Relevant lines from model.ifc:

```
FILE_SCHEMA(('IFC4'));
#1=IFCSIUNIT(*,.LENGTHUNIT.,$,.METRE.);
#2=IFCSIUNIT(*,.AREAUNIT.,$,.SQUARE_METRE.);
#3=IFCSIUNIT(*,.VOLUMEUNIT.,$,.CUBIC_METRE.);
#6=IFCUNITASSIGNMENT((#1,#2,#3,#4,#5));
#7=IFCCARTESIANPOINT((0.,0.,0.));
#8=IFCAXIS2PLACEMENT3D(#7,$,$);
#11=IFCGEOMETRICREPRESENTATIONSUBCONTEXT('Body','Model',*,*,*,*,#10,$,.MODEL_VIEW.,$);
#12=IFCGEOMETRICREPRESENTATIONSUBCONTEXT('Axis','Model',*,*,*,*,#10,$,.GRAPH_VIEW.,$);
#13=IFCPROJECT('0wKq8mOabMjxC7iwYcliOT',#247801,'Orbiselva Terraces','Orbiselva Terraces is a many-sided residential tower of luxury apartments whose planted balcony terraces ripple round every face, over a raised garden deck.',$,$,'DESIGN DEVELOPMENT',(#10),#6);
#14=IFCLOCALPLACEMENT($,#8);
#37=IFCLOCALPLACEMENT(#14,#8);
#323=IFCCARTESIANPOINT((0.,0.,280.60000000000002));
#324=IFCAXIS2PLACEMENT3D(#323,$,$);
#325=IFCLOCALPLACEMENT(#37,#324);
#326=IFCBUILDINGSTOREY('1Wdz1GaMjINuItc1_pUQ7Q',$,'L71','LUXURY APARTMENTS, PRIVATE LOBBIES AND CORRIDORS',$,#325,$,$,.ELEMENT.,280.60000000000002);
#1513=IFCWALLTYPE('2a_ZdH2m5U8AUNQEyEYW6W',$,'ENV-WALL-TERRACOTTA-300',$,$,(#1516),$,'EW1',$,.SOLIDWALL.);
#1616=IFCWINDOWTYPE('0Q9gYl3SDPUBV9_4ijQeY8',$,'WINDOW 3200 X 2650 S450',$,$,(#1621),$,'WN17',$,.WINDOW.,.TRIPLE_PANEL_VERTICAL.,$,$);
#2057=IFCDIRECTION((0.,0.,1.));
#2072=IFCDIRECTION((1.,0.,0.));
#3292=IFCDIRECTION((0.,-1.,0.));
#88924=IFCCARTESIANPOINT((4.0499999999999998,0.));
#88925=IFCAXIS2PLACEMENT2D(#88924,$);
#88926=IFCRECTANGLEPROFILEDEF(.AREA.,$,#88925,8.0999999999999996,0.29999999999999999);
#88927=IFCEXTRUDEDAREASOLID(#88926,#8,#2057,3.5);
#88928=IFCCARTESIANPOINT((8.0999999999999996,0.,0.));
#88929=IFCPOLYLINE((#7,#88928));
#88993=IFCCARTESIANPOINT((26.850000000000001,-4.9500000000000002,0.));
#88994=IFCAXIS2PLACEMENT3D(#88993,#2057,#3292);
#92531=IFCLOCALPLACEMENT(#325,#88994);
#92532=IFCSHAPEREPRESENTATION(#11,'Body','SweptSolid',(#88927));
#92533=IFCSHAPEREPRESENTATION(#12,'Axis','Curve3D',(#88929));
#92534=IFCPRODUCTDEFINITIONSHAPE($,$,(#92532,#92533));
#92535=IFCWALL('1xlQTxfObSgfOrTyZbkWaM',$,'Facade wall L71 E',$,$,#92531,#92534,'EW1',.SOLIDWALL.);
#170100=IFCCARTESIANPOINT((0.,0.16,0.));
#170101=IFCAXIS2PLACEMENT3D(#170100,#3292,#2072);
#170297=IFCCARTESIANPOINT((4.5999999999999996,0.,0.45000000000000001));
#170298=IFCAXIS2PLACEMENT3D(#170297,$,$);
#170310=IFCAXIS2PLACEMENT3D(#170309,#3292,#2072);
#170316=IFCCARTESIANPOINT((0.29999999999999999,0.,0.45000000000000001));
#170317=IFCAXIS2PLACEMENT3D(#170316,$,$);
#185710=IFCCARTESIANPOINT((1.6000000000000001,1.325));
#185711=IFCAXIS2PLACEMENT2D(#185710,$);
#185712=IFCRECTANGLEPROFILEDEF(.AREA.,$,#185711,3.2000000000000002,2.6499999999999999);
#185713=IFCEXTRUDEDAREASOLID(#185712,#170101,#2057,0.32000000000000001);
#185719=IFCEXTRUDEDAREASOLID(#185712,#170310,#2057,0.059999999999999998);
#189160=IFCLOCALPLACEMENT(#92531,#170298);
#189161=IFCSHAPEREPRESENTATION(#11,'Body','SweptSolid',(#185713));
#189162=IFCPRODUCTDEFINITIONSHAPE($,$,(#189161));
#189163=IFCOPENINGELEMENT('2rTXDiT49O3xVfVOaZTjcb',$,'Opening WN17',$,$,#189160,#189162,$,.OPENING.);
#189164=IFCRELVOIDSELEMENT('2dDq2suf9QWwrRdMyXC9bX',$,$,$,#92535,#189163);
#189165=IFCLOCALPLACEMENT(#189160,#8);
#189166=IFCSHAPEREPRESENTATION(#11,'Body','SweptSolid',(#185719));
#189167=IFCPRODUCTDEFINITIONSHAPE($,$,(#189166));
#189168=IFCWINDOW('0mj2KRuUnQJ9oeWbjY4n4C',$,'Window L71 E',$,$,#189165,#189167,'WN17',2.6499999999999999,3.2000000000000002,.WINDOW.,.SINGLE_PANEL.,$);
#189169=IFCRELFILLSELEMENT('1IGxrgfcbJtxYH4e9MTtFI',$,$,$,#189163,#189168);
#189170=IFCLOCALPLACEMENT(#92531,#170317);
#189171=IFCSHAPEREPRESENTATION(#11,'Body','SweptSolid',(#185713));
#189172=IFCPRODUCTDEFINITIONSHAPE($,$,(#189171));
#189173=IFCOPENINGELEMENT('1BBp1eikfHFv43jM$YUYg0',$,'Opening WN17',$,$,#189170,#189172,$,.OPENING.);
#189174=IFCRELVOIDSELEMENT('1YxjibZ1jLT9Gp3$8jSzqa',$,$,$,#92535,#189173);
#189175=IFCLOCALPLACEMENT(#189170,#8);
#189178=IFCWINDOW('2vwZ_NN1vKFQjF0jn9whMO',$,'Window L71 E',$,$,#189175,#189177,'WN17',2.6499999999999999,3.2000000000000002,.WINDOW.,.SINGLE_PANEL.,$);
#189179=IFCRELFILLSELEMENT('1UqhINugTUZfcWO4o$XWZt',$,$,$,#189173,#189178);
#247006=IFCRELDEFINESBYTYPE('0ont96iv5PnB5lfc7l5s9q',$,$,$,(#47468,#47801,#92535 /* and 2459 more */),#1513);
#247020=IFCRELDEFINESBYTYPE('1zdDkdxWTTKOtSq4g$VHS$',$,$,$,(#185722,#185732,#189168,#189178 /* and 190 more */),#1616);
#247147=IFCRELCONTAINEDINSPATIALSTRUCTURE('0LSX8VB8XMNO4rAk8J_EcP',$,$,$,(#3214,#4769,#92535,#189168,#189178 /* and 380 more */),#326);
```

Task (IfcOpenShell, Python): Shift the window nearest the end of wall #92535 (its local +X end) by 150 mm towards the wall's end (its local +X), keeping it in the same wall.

```python
import ifcopenshell
import ifcopenshell.api.geometry
import ifcopenshell.util.placement
import ifcopenshell.util.unit

model = ifcopenshell.open("model.ifc")
unit_scale = ifcopenshell.util.unit.calculate_unit_scale(model)

window = model.by_guid("0mj2KRuUnQJ9oeWbjY4n4C")
opening = window.FillsVoids[0].RelatingOpeningElement
wall = opening.VoidsElements[0].RelatingBuildingElement

wall_matrix = ifcopenshell.util.placement.get_local_placement(wall.ObjectPlacement)
shift = wall_matrix[:3, 0] * 0.15 / unit_scale
before = ifcopenshell.util.placement.get_local_placement(window.ObjectPlacement)[:3, 3].copy()

# The window is placed relative to its opening, so it follows when the opening moves.
matrix = ifcopenshell.util.placement.get_local_placement(opening.ObjectPlacement)
matrix[:3, 3] += shift
ifcopenshell.api.geometry.edit_object_placement(
    model, product=opening, matrix=matrix, is_si=False, should_transform_children=True
)

after = ifcopenshell.util.placement.get_local_placement(window.ObjectPlacement)[:3, 3]
print("window moved by", (after - before).round(3) + 0.0)

model.write("model-out.ifc")
```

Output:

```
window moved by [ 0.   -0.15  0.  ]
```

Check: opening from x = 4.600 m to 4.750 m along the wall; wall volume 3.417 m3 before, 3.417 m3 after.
